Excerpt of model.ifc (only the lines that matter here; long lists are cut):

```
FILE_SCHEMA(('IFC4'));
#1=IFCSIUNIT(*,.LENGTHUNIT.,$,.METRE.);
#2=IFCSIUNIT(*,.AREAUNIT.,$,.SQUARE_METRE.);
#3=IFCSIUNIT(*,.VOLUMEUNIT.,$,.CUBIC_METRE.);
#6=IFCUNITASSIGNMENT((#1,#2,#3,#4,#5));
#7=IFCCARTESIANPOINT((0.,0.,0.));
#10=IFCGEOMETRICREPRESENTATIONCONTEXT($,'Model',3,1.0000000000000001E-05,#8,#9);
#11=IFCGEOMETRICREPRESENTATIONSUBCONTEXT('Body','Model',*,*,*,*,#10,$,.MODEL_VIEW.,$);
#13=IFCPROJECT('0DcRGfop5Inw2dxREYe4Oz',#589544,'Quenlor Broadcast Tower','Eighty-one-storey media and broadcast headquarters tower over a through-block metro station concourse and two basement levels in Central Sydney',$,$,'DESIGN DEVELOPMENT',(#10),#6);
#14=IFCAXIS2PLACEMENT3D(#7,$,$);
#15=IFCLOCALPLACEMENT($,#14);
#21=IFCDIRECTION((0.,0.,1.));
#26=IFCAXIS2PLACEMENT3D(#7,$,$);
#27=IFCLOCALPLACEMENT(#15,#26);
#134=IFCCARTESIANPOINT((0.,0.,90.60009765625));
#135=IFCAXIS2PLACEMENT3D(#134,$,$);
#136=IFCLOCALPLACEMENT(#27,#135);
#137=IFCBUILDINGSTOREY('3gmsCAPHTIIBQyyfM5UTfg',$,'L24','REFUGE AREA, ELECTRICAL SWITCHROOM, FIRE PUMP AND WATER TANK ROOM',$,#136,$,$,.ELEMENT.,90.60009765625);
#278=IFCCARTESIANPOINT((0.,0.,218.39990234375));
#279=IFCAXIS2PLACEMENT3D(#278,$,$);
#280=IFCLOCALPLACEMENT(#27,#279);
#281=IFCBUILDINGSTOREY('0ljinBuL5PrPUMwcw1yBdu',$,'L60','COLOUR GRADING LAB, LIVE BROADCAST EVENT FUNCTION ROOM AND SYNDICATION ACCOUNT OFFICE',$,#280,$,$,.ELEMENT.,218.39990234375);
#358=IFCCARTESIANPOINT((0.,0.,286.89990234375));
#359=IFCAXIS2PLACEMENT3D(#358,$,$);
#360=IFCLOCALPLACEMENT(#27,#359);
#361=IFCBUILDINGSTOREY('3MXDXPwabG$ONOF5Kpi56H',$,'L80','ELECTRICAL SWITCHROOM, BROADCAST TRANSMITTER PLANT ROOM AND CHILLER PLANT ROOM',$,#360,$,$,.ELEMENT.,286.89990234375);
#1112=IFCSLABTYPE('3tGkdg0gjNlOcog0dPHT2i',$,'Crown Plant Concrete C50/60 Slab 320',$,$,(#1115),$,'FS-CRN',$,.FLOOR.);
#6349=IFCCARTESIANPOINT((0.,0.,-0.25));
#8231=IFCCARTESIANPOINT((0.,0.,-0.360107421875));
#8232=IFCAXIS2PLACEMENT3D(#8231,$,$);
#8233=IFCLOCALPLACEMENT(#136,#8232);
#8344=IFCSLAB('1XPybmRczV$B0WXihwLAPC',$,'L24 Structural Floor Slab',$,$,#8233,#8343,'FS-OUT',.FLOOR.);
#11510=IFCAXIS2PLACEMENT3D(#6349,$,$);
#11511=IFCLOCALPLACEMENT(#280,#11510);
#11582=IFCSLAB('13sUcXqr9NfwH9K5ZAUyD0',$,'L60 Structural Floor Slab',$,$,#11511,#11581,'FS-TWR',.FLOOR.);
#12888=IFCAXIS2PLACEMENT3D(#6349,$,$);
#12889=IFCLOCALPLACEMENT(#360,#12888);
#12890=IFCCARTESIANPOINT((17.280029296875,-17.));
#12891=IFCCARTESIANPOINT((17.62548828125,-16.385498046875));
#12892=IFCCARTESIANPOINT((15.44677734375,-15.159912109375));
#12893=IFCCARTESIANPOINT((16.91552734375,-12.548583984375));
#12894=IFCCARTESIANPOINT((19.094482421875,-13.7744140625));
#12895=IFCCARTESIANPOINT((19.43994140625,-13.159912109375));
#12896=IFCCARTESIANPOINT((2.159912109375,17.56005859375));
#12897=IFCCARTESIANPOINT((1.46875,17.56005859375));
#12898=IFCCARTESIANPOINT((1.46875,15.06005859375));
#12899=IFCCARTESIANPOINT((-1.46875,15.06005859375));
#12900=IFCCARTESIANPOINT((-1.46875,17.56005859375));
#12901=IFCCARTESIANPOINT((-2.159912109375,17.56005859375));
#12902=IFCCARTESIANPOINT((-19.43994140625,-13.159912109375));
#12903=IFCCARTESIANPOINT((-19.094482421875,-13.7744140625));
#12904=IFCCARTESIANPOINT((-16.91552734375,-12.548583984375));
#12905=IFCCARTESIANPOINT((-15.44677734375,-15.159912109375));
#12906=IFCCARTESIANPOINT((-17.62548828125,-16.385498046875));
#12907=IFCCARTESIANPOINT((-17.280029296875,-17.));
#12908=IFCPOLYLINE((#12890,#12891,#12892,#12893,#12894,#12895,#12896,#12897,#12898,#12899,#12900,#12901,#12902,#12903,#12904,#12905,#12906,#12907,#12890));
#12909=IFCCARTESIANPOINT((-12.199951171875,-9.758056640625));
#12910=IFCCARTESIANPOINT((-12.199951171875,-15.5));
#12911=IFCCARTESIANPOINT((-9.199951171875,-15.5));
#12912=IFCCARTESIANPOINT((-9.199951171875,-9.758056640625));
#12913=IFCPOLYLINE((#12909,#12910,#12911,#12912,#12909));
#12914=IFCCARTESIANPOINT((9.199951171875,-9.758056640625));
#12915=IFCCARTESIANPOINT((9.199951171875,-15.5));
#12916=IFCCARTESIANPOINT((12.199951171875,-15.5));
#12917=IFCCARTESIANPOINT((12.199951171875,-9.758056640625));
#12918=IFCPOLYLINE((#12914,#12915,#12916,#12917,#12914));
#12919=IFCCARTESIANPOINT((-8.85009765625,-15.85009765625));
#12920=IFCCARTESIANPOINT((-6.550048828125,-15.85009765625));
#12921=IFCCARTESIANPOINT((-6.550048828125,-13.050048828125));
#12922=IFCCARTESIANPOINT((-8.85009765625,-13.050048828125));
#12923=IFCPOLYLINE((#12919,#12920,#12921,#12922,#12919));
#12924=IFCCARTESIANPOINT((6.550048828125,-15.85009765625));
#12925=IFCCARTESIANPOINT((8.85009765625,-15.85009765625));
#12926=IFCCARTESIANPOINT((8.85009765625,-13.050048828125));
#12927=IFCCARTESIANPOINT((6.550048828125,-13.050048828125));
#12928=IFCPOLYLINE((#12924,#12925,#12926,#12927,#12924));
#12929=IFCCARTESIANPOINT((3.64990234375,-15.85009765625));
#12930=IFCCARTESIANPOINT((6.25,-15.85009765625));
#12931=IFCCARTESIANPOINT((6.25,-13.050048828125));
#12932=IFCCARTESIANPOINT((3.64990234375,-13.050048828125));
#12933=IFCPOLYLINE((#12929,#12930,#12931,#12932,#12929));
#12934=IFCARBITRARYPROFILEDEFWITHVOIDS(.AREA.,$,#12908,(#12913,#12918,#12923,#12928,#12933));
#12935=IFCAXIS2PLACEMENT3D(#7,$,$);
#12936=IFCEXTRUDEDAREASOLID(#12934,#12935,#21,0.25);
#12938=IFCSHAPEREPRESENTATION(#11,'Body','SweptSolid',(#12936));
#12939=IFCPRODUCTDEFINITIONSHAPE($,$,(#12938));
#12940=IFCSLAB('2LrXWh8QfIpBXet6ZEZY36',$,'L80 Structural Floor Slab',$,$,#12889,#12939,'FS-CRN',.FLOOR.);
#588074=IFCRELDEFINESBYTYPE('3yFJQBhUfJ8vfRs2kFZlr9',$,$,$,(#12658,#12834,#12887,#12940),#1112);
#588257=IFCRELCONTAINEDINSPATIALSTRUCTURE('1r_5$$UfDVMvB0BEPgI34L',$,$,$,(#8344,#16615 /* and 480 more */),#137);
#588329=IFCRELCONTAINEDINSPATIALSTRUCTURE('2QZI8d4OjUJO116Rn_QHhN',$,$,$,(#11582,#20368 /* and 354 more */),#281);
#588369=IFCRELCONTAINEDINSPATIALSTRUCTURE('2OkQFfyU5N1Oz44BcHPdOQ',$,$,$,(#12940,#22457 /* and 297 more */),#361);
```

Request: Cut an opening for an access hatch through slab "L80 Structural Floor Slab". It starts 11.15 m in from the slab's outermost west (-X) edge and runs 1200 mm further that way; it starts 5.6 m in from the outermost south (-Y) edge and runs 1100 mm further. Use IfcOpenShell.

```python
import numpy as np
import ifcopenshell
import ifcopenshell.api.feature
import ifcopenshell.api.geometry
import ifcopenshell.api.root
import ifcopenshell.geom
import ifcopenshell.util.placement
import ifcopenshell.util.representation
import ifcopenshell.util.shape
import ifcopenshell.util.unit

model = ifcopenshell.open("model.ifc")
unit_scale = ifcopenshell.util.unit.calculate_unit_scale(model)
settings = ifcopenshell.geom.settings()


def volume(element):
    """Net volume in cubic metres, openings subtracted."""
    shape = ifcopenshell.geom.create_shape(settings, element)
    return ifcopenshell.util.shape.get_volume(shape.geometry)


slab = model.by_guid("2LrXWh8QfIpBXet6ZEZY36")
before = volume(slab)

# Extent in the slab's own axes, in metres. The edges named are its -X and -Y sides.
slab_shape = ifcopenshell.geom.create_shape(settings, slab)
vertices = ifcopenshell.util.shape.get_vertices(slab_shape.geometry)
x_min, y_min, bottom = vertices.min(axis=0)
top = vertices[:, 2].max()

opening = ifcopenshell.api.root.create_entity(model, ifc_class="IfcOpeningElement", name="Access hatch opening", predefined_type="OPENING")
context = ifcopenshell.util.representation.get_context(model, "Model", "Body", "MODEL_VIEW")
width, depth = 1.2, 1.1
outline = [(0.0, 0.0), (width, 0.0), (width, depth), (0.0, depth), (0.0, 0.0)]
# Overshoot both faces by 50 mm so the cut is clean.
shape = ifcopenshell.api.geometry.add_slab_representation(
    model, context=context, depth=top - bottom + 0.1, polyline=outline
)
ifcopenshell.api.geometry.assign_representation(model, product=opening, representation=shape)

matrix = ifcopenshell.util.placement.get_local_placement(slab.ObjectPlacement)
matrix[:, 3] = matrix @ np.append(np.array([x_min + 11.15, y_min + 5.6, bottom - 0.05]) / unit_scale, 1.0)
ifcopenshell.api.geometry.edit_object_placement(model, product=opening, matrix=matrix, is_si=False)
ifcopenshell.api.feature.add_feature(model, feature=opening, element=slab)

after = volume(slab)

print(f"slab volume {before:.3f} -> {after:.3f} m3")

model.write("model_v2.ifc")
```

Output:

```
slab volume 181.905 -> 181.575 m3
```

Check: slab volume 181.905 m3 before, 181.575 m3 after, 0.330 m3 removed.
